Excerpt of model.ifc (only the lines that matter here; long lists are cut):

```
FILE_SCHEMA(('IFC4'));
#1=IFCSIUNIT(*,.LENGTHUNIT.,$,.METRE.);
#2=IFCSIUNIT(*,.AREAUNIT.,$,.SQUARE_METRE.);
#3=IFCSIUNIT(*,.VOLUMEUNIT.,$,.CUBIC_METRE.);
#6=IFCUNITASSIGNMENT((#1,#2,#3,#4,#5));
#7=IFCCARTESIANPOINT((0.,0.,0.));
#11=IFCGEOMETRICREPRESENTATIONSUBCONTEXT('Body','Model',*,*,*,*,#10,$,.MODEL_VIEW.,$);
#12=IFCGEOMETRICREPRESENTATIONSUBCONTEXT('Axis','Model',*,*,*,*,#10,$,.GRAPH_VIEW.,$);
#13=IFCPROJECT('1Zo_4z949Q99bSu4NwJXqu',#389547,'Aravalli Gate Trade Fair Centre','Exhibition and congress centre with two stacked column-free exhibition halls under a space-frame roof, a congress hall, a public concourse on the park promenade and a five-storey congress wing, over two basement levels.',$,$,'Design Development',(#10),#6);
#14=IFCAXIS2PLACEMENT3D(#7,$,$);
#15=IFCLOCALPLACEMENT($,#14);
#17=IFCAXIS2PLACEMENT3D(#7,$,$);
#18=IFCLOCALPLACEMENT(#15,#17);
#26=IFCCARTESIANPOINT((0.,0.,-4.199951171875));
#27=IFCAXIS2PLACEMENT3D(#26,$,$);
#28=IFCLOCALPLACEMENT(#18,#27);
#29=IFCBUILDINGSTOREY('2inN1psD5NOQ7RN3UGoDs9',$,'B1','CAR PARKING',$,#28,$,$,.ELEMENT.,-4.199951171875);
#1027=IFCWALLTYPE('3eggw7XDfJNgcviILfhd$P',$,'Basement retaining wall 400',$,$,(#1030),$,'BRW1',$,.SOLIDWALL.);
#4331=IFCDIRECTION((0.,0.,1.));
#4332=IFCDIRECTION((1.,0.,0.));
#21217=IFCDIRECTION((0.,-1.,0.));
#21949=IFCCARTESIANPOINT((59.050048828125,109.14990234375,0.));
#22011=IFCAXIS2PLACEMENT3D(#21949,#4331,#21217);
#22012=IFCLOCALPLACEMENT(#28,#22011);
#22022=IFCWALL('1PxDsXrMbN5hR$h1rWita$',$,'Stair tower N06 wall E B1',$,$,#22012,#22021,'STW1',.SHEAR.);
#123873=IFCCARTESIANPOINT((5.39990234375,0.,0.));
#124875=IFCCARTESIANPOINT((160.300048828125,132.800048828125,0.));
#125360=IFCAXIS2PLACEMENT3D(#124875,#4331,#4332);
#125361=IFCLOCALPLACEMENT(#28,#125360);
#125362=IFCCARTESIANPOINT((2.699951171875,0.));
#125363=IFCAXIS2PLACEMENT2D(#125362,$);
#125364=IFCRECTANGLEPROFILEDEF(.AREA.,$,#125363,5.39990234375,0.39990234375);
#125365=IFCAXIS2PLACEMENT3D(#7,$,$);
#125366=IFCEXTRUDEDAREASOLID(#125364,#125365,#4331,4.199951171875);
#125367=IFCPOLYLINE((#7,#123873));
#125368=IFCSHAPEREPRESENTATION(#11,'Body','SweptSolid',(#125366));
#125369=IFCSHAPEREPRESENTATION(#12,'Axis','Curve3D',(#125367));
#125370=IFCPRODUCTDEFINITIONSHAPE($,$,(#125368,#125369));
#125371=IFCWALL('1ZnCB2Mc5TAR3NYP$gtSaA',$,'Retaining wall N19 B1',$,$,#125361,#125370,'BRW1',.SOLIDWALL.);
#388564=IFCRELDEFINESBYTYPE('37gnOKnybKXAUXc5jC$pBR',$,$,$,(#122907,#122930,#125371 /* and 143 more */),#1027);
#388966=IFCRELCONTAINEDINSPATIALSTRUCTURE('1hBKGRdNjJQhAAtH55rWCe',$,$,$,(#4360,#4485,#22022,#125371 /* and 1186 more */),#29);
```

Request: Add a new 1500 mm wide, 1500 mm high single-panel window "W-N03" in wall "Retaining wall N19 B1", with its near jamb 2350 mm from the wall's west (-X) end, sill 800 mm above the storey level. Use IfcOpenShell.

```python
import numpy as np
import ifcopenshell
import ifcopenshell.api.feature
import ifcopenshell.api.geometry
import ifcopenshell.api.root
import ifcopenshell.api.spatial
import ifcopenshell.geom
import ifcopenshell.util.element
import ifcopenshell.util.placement
import ifcopenshell.util.representation
import ifcopenshell.util.shape
import ifcopenshell.util.unit

model = ifcopenshell.open("model.ifc")
unit_scale = ifcopenshell.util.unit.calculate_unit_scale(model)
settings = ifcopenshell.geom.settings()


def volume(element):
    """Net volume in cubic metres, openings subtracted."""
    shape = ifcopenshell.geom.create_shape(settings, element)
    return ifcopenshell.util.shape.get_volume(shape.geometry)


wall = model.by_id(125371)
storey = ifcopenshell.util.element.get_container(wall, ifc_class="IfcBuildingStorey")
context = ifcopenshell.util.representation.get_context(model, "Model", "Body", "MODEL_VIEW")
before = volume(wall)

width, height, from_end, sill = 1.5, 1.5, 2.35, 0.8  # metres

# The wall runs along its own X axis, and the end named is its -X end.
wall_shape = ifcopenshell.geom.create_shape(settings, wall)
x, y, z = ifcopenshell.util.shape.get_vertices(wall_shape.geometry).T
start = x.min() + from_end
face, thickness = float(y.min()), float(y.max() - y.min())
wall_matrix = ifcopenshell.util.placement.get_local_placement(wall.ObjectPlacement)
level = ifcopenshell.util.placement.get_local_placement(storey.ObjectPlacement)[2, 3]


def in_wall(x, y):
    """Placement at x, y metres in the wall's axes, at sill height."""
    matrix = wall_matrix.copy()
    matrix[:, 3] = wall_matrix @ np.array([x / unit_scale, y / unit_scale, 0.0, 1.0])
    matrix[2, 3] = level + sill / unit_scale
    return matrix


# Opening: a box that overshoots both wall faces by 50 mm.
opening = ifcopenshell.api.root.create_entity(model, ifc_class="IfcOpeningElement", predefined_type="OPENING")
box = ifcopenshell.api.geometry.add_wall_representation(
    model, context=context, length=width, height=height, thickness=thickness + 0.1
)
ifcopenshell.api.geometry.assign_representation(model, product=opening, representation=box)
ifcopenshell.api.geometry.edit_object_placement(model, product=opening, matrix=in_wall(start, face - 0.05), is_si=False)
ifcopenshell.api.feature.add_feature(model, feature=opening, element=wall)

window = ifcopenshell.api.root.create_entity(model, ifc_class="IfcWindow", name="W-N03", predefined_type="WINDOW")
window.OverallWidth, window.OverallHeight = width / unit_scale, height / unit_scale
window.PartitioningType = "SINGLE_PANEL"
body = ifcopenshell.api.geometry.add_window_representation(
    model,
    context=context,
    overall_width=window.OverallWidth,
    overall_height=window.OverallHeight,
    partition_type="SINGLE_PANEL",
)
ifcopenshell.api.geometry.assign_representation(model, product=window, representation=body)
ifcopenshell.api.spatial.assign_container(model, products=[window], relating_structure=storey)
ifcopenshell.api.feature.add_filling(model, opening=opening, element=window)

# Centre the window in the wall's thickness.
ifcopenshell.api.geometry.edit_object_placement(model, product=window, matrix=in_wall(start, face), is_si=False)
window_shape = ifcopenshell.geom.create_shape(settings, window)
depth = ifcopenshell.util.shape.get_vertices(window_shape.geometry)[:, 1]
offset = face + thickness / 2 - (depth.min() + depth.max()) / 2
ifcopenshell.api.geometry.edit_object_placement(model, product=window, matrix=in_wall(start, offset), is_si=False)

after = volume(wall)

print(f"wall volume {before:.3f} -> {after:.3f} m3")

model.write("model_rev.ifc")
```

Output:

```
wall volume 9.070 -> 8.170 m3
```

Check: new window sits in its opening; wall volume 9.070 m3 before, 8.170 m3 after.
